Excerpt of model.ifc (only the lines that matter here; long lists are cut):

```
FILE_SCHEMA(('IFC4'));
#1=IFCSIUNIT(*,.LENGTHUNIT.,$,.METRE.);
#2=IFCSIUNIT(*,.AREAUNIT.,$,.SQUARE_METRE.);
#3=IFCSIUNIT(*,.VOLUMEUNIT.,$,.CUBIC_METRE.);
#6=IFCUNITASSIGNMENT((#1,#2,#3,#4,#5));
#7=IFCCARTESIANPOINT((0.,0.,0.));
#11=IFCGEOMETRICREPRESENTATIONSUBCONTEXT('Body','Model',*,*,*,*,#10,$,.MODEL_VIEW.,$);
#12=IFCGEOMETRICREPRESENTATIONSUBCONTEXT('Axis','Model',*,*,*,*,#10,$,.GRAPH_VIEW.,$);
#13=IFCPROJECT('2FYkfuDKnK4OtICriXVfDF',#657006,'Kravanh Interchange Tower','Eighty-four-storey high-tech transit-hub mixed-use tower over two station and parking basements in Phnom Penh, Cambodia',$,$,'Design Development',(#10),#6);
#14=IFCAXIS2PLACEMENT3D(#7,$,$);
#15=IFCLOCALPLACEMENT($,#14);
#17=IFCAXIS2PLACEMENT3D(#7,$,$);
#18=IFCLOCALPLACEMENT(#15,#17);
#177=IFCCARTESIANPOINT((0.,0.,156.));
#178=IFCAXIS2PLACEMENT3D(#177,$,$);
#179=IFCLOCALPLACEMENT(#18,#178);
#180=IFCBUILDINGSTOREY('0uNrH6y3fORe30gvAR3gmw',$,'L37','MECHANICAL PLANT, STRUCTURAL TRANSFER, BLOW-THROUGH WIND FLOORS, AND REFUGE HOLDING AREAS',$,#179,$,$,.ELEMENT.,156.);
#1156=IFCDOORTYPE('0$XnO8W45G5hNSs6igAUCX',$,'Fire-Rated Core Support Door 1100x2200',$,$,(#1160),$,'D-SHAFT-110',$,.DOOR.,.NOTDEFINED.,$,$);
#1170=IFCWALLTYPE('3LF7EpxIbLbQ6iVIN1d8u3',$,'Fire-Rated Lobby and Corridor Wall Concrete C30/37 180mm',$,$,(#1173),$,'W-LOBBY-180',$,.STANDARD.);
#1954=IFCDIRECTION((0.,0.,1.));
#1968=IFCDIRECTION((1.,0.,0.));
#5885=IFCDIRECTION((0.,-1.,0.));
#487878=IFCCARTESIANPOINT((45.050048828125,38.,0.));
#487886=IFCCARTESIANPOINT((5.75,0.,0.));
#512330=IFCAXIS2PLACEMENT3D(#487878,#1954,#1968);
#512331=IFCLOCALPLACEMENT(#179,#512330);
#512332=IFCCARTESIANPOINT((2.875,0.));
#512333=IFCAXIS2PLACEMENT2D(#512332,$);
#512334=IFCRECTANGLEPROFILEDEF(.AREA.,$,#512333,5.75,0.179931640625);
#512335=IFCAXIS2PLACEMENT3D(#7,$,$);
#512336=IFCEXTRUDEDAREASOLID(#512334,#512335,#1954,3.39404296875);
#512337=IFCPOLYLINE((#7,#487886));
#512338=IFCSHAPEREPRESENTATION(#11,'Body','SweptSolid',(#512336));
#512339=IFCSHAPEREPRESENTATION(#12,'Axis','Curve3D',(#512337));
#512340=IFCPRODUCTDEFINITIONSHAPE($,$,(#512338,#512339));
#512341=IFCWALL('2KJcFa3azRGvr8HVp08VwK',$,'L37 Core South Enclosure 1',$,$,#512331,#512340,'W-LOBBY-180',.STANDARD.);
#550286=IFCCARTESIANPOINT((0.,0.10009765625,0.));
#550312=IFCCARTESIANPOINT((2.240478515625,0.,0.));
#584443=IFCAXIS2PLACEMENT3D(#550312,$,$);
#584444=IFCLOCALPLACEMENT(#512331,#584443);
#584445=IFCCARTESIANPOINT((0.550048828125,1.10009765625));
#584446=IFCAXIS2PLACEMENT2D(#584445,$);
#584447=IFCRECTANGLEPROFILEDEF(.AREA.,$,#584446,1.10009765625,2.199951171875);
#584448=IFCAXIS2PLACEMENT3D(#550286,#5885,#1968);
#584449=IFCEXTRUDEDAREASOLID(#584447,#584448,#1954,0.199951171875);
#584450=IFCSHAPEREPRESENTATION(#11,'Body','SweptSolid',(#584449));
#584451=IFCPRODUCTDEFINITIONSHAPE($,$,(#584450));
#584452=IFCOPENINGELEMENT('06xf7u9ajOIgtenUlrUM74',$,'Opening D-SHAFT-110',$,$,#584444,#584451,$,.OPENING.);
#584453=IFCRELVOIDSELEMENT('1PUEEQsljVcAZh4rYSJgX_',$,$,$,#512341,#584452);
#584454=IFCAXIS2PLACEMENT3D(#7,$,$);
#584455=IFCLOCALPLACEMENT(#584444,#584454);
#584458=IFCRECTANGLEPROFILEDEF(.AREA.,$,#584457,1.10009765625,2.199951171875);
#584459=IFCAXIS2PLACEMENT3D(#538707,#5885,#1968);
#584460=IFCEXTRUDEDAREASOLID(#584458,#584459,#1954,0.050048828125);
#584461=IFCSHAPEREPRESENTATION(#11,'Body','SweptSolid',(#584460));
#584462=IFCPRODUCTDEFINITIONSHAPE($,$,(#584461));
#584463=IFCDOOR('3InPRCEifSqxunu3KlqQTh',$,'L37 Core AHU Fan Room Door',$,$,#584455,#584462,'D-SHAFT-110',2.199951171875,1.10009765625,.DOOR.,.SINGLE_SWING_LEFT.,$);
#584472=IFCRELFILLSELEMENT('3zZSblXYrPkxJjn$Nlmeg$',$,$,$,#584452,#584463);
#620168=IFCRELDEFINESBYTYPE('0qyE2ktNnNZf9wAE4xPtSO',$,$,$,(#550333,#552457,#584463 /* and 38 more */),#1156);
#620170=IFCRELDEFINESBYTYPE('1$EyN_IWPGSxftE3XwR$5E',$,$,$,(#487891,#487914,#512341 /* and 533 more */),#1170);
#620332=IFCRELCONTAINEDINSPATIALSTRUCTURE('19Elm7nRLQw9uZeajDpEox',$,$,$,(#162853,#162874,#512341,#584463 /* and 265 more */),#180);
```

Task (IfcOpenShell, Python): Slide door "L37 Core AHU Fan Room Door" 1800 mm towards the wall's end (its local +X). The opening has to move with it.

```python
import ifcopenshell
import ifcopenshell.api.geometry
import ifcopenshell.util.placement
import ifcopenshell.util.unit

model = ifcopenshell.open("model.ifc")
unit_scale = ifcopenshell.util.unit.calculate_unit_scale(model)

door = model.by_guid("3InPRCEifSqxunu3KlqQTh")
opening = door.FillsVoids[0].RelatingOpeningElement
wall = opening.VoidsElements[0].RelatingBuildingElement

wall_matrix = ifcopenshell.util.placement.get_local_placement(wall.ObjectPlacement)
shift = wall_matrix[:3, 0] * 1.8 / unit_scale
before = ifcopenshell.util.placement.get_local_placement(door.ObjectPlacement)[:3, 3].copy()

# The door is placed relative to its opening, so it follows when the opening moves.
matrix = ifcopenshell.util.placement.get_local_placement(opening.ObjectPlacement)
matrix[:3, 3] += shift
ifcopenshell.api.geometry.edit_object_placement(
    model, product=opening, matrix=matrix, is_si=False, should_transform_children=True
)

after = ifcopenshell.util.placement.get_local_placement(door.ObjectPlacement)[:3, 3]
print("door moved by", (after - before).round(3) + 0.0)

model.write("model-out.ifc")
```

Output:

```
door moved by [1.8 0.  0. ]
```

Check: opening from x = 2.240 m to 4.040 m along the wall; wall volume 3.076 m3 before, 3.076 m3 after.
